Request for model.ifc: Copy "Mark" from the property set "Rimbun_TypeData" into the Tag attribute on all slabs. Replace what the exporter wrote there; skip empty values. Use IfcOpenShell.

First a look at what the model holds.

```python
import ifcopenshell
import ifcopenshell.util.element

model = ifcopenshell.open("model.ifc")
print(model.schema)
slabs = model.by_type("IfcSlab")
print(len(slabs), "slabs")
for e in slabs[:8]:
    source = ifcopenshell.util.element.get_pset(e, "Rimbun_TypeData", "Mark")
    target = e.Tag
    print(e.id(), repr(source), repr(target), sep=" | ")
```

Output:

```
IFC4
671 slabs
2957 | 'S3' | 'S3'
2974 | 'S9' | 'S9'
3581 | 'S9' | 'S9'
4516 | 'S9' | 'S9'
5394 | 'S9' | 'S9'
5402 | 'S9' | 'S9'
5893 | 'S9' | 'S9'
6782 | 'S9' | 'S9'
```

```python
import ifcopenshell
import ifcopenshell.util.element

model = ifcopenshell.open("model.ifc")

count = 0
for e in model.by_type("IfcSlab"):
    value = ifcopenshell.util.element.get_pset(e, "Rimbun_TypeData", "Mark")
    current = e.Tag
    if not value or not value.strip() or current == value:
        continue
    e.Tag = value
    count += 1

print(count, "slabs updated")

model.write("model-out.ifc")
```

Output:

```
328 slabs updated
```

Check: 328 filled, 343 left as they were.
